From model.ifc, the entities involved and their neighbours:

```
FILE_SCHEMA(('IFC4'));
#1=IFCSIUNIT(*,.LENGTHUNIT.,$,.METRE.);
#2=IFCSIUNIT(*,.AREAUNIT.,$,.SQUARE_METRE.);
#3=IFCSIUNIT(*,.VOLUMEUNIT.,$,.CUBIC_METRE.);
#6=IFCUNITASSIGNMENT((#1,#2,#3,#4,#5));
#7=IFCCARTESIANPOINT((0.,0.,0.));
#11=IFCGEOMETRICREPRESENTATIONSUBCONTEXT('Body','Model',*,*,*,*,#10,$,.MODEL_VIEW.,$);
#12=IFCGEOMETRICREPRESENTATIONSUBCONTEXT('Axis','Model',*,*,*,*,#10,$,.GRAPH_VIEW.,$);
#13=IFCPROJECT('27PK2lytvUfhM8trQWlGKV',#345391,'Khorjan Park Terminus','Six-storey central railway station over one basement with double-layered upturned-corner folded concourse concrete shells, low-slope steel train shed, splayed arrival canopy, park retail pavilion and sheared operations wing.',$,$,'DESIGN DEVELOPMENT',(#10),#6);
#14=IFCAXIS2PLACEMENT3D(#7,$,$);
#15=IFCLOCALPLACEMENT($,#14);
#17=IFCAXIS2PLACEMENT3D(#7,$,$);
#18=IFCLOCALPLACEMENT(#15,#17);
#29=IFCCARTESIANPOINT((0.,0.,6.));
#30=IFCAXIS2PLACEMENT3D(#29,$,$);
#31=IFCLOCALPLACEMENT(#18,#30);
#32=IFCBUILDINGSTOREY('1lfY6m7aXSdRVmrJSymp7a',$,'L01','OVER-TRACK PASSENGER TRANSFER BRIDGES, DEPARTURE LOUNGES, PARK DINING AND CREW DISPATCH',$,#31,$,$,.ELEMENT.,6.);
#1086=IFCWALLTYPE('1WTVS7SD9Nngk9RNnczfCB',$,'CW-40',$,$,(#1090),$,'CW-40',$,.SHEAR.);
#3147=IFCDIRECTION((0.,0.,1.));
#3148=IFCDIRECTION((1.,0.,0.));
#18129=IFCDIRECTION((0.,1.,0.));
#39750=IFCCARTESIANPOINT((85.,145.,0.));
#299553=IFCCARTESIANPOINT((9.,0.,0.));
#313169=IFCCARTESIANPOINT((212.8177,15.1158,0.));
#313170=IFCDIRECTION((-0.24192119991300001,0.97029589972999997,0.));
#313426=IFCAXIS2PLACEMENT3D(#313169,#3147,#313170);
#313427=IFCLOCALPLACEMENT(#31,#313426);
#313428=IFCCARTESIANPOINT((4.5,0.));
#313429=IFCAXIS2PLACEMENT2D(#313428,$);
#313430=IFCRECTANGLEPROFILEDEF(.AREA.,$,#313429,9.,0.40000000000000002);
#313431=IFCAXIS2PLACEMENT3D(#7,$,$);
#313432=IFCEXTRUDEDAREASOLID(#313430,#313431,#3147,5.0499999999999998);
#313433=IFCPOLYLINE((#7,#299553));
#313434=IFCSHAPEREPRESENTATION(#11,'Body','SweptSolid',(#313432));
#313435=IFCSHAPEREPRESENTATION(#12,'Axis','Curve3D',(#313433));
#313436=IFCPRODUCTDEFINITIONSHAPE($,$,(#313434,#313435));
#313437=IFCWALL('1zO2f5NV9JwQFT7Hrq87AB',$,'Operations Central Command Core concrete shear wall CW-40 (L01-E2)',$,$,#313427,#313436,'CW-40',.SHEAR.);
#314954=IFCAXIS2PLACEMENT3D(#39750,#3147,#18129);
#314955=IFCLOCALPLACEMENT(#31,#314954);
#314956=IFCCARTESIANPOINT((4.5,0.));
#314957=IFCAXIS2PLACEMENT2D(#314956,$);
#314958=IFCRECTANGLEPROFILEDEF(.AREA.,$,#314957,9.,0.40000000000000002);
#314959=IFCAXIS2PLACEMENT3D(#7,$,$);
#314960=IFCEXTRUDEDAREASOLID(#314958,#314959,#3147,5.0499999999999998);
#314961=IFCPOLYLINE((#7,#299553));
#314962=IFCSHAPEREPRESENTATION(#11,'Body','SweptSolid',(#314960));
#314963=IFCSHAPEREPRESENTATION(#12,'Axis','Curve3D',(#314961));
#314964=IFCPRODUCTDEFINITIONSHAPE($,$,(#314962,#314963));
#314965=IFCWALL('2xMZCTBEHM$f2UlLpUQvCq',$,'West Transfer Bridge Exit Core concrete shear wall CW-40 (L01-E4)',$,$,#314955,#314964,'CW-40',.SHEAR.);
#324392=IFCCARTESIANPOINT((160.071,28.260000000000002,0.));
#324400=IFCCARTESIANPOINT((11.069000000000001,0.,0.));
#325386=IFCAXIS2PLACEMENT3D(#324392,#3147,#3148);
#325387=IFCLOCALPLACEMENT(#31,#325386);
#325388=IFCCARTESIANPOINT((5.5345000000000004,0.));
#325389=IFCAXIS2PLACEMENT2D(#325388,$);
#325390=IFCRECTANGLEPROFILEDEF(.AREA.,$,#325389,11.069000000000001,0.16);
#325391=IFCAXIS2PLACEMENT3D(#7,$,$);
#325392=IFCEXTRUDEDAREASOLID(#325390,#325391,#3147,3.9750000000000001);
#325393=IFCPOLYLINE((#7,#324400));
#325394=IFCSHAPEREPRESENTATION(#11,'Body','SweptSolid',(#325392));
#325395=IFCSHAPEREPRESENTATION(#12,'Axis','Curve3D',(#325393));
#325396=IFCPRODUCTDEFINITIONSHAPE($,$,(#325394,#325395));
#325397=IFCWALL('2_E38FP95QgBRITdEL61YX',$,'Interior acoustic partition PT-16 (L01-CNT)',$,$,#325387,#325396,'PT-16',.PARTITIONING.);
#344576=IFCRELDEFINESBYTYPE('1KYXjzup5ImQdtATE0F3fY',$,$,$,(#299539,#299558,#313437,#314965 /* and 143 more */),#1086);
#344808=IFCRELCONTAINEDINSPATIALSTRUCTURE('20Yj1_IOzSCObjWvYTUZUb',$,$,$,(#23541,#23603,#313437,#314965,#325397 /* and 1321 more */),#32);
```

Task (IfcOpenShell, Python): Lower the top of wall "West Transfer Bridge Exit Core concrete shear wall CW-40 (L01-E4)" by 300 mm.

```python
import ifcopenshell
import ifcopenshell.geom
import ifcopenshell.util.representation
import ifcopenshell.util.shape

model = ifcopenshell.open("model.ifc")
settings = ifcopenshell.geom.settings()


def volume(element):
    """Net volume in cubic metres, openings subtracted."""
    shape = ifcopenshell.geom.create_shape(settings, element)
    return ifcopenshell.util.shape.get_volume(shape.geometry)


wall = model.by_guid("2xMZCTBEHM$f2UlLpUQvCq")
before = volume(wall)

body = ifcopenshell.util.representation.get_representation(wall, "Model", "Body")
solid = body.Items[0]
old_height = solid.Depth
solid.Depth -= 0.3
after = volume(wall)

print(f"height {old_height:g} -> {solid.Depth:g}, volume {before:.3f} -> {after:.3f} m3")

model.write("model_rev.ifc")
```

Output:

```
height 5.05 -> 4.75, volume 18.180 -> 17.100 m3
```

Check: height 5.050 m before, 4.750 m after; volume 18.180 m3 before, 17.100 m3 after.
